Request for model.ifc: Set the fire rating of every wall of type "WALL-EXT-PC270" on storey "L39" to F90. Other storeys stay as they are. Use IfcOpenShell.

First a look at what the model holds.

```python
import ifcopenshell
import ifcopenshell.util.element

model = ifcopenshell.open("model.ifc")
print(model.schema)
storey = next(s for s in model.by_type("IfcBuildingStorey") if s.Name == "L39")
walls = [e for e in ifcopenshell.util.element.get_decomposition(storey) if e.is_a("IfcWall")]
seen = {}
for e in walls:
    element_type = ifcopenshell.util.element.get_type(e)
    key = (element_type.Name if element_type != e and element_type else None, ifcopenshell.util.element.get_pset(e, "Pset_WallCommon", "FireRating"))
    seen[key] = seen.get(key, 0) + 1
for (name, value), count in sorted(seen.items(), key=str):
    print(count, "x", name, "|", value)
```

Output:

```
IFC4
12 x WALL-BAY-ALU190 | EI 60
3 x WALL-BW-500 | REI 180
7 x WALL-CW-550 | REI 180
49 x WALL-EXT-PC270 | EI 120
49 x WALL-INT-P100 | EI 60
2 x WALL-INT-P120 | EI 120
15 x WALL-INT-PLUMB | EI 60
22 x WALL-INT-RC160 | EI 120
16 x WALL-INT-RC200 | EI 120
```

```python
import ifcopenshell
import ifcopenshell.api.pset
import ifcopenshell.util.element

model = ifcopenshell.open("model.ifc")

storey = next(s for s in model.by_type("IfcBuildingStorey") if s.Name == "L39")
walls = [e for e in ifcopenshell.util.element.get_decomposition(storey) if e.is_a("IfcWall")]

count = 0
for e in walls:
    element_type = ifcopenshell.util.element.get_type(e)
    if element_type in (None, e) or element_type.Name != "WALL-EXT-PC270":
        continue
    found = ifcopenshell.util.element.get_pset(e, "Pset_WallCommon", should_inherit=False)
    if found:
        pset = model.by_id(found["id"])
        if len(ifcopenshell.util.element.get_elements_by_pset(pset)) > 1:
            pset = ifcopenshell.api.pset.unshare_pset(model, products=[e], pset=pset)[0]
    else:
        pset = ifcopenshell.api.pset.add_pset(model, product=e, name="Pset_WallCommon")
    ifcopenshell.api.pset.edit_pset(model, pset=pset, properties={"FireRating": "F90"})
    count += 1

print(count, "walls updated")

model.write("model_rev.ifc")
```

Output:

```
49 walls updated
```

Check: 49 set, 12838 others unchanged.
